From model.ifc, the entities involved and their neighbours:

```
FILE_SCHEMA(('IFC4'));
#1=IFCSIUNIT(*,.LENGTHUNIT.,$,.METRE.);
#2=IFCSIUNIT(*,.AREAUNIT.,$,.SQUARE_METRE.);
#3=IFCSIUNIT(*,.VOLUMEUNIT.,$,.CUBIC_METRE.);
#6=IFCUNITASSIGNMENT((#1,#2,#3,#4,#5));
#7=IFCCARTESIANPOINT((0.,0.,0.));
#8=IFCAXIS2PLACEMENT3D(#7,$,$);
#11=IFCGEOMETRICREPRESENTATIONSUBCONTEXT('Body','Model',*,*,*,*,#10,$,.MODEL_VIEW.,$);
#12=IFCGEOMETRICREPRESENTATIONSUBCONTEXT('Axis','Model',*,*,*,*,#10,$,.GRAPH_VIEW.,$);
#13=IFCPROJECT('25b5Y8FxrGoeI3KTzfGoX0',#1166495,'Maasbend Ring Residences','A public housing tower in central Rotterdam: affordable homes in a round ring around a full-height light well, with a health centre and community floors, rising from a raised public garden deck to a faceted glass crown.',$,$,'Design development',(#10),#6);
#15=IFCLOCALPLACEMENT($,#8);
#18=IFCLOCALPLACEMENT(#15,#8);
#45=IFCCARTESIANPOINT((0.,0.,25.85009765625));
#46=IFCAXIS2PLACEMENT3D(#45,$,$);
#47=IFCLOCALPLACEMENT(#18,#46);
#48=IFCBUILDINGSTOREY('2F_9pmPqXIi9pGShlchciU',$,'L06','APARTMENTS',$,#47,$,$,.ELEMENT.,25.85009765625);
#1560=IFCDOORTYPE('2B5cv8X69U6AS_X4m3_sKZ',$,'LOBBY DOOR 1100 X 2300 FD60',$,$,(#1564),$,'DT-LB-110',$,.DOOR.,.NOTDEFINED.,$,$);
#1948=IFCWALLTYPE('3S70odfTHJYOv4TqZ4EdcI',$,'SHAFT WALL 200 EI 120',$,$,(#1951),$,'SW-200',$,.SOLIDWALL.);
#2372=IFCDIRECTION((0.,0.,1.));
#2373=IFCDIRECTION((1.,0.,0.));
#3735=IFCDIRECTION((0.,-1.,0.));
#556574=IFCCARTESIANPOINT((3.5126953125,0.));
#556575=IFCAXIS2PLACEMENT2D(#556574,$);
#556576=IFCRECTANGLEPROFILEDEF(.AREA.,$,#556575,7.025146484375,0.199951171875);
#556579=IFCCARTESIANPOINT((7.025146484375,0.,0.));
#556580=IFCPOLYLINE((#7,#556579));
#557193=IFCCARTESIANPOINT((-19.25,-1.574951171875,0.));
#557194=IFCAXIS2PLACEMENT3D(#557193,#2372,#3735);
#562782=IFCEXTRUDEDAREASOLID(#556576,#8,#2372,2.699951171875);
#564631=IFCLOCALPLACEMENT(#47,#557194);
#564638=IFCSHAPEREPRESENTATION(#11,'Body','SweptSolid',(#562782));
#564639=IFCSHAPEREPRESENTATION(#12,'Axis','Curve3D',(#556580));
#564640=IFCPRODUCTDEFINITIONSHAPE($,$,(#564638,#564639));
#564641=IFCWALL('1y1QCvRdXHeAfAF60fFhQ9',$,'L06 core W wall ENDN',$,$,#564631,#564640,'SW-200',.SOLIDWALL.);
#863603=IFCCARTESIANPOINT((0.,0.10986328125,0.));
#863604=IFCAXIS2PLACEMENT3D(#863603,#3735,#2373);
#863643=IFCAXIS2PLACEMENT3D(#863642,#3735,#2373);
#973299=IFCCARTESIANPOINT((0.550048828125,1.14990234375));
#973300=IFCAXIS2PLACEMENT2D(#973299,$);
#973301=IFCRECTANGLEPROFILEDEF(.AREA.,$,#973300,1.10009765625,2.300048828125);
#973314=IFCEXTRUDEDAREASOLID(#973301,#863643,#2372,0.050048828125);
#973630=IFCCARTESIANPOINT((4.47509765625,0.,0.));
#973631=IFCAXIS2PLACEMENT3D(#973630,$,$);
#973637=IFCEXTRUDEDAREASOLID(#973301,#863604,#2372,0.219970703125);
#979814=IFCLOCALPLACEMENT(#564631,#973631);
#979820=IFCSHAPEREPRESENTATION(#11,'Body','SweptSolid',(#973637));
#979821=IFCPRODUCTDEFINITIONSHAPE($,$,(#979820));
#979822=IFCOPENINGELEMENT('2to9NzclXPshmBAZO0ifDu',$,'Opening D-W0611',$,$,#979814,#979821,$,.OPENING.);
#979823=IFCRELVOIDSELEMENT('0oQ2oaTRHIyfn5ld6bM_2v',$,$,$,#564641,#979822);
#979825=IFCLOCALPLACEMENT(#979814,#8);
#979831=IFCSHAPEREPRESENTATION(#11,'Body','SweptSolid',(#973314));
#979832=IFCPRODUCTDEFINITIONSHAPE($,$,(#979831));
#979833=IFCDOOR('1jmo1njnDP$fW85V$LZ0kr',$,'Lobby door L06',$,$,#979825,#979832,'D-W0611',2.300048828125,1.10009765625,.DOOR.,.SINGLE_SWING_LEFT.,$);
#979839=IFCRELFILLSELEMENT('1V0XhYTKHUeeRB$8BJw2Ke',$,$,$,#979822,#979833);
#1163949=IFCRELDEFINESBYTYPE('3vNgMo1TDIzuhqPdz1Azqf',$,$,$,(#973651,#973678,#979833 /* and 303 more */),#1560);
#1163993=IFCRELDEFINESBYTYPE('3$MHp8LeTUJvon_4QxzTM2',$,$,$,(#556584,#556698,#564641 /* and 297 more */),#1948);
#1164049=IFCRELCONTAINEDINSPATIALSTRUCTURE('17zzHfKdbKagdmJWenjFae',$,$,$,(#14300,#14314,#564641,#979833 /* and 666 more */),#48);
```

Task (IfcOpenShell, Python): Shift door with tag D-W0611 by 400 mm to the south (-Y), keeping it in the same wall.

```python
import ifcopenshell
import ifcopenshell.api.geometry
import ifcopenshell.util.placement
import ifcopenshell.util.unit

model = ifcopenshell.open("model.ifc")
unit_scale = ifcopenshell.util.unit.calculate_unit_scale(model)

door = model.by_guid("1jmo1njnDP$fW85V$LZ0kr")
opening = door.FillsVoids[0].RelatingOpeningElement
wall = opening.VoidsElements[0].RelatingBuildingElement

wall_matrix = ifcopenshell.util.placement.get_local_placement(wall.ObjectPlacement)
shift = wall_matrix[:3, 0] * 0.4 / unit_scale
before = ifcopenshell.util.placement.get_local_placement(door.ObjectPlacement)[:3, 3].copy()

# The door is placed relative to its opening, so it follows when the opening moves.
matrix = ifcopenshell.util.placement.get_local_placement(opening.ObjectPlacement)
matrix[:3, 3] += shift
ifcopenshell.api.geometry.edit_object_placement(
    model, product=opening, matrix=matrix, is_si=False, should_transform_children=True
)

after = ifcopenshell.util.placement.get_local_placement(door.ObjectPlacement)[:3, 3]
print("door moved by", (after - before).round(3) + 0.0)

model.write("model_v2.ifc")
```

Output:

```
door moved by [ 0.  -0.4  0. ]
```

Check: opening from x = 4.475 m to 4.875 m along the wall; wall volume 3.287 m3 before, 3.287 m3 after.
